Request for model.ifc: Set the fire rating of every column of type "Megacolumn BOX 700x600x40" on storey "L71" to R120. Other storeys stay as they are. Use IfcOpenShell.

First a look at what the model holds.

```python
import ifcopenshell
import ifcopenshell.util.element

model = ifcopenshell.open("model.ifc")
print(model.schema)
storey = next(s for s in model.by_type("IfcBuildingStorey") if s.Name == "L71")
columns = [e for e in ifcopenshell.util.element.get_decomposition(storey) if e.is_a("IfcColumn")]
seen = {}
for e in columns:
    element_type = ifcopenshell.util.element.get_type(e)
    key = (element_type.Name if element_type != e and element_type else None, ifcopenshell.util.element.get_pset(e, "Pset_ColumnCommon", "FireRating"))
    seen[key] = seen.get(key, 0) + 1
for (name, value), count in sorted(seen.items(), key=str):
    print(count, "x", name, "|", value)
```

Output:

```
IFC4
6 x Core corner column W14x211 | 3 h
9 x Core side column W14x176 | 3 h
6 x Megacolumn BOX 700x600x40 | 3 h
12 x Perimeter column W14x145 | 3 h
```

```python
import ifcopenshell
import ifcopenshell.api.pset
import ifcopenshell.util.element

model = ifcopenshell.open("model.ifc")

storey = next(s for s in model.by_type("IfcBuildingStorey") if s.Name == "L71")
columns = [e for e in ifcopenshell.util.element.get_decomposition(storey) if e.is_a("IfcColumn")]

count = 0
for e in columns:
    element_type = ifcopenshell.util.element.get_type(e)
    if element_type in (None, e) or element_type.Name != "Megacolumn BOX 700x600x40":
        continue
    found = ifcopenshell.util.element.get_pset(e, "Pset_ColumnCommon", should_inherit=False)
    if found:
        pset = model.by_id(found["id"])
        if len(ifcopenshell.util.element.get_elements_by_pset(pset)) > 1:
            pset = ifcopenshell.api.pset.unshare_pset(model, products=[e], pset=pset)[0]
    else:
        pset = ifcopenshell.api.pset.add_pset(model, product=e, name="Pset_ColumnCommon")
    ifcopenshell.api.pset.edit_pset(model, pset=pset, properties={"FireRating": "R120"})
    count += 1

print(count, "columns updated")

model.write("model_updated.ifc")
```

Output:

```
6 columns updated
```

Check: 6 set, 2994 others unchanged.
